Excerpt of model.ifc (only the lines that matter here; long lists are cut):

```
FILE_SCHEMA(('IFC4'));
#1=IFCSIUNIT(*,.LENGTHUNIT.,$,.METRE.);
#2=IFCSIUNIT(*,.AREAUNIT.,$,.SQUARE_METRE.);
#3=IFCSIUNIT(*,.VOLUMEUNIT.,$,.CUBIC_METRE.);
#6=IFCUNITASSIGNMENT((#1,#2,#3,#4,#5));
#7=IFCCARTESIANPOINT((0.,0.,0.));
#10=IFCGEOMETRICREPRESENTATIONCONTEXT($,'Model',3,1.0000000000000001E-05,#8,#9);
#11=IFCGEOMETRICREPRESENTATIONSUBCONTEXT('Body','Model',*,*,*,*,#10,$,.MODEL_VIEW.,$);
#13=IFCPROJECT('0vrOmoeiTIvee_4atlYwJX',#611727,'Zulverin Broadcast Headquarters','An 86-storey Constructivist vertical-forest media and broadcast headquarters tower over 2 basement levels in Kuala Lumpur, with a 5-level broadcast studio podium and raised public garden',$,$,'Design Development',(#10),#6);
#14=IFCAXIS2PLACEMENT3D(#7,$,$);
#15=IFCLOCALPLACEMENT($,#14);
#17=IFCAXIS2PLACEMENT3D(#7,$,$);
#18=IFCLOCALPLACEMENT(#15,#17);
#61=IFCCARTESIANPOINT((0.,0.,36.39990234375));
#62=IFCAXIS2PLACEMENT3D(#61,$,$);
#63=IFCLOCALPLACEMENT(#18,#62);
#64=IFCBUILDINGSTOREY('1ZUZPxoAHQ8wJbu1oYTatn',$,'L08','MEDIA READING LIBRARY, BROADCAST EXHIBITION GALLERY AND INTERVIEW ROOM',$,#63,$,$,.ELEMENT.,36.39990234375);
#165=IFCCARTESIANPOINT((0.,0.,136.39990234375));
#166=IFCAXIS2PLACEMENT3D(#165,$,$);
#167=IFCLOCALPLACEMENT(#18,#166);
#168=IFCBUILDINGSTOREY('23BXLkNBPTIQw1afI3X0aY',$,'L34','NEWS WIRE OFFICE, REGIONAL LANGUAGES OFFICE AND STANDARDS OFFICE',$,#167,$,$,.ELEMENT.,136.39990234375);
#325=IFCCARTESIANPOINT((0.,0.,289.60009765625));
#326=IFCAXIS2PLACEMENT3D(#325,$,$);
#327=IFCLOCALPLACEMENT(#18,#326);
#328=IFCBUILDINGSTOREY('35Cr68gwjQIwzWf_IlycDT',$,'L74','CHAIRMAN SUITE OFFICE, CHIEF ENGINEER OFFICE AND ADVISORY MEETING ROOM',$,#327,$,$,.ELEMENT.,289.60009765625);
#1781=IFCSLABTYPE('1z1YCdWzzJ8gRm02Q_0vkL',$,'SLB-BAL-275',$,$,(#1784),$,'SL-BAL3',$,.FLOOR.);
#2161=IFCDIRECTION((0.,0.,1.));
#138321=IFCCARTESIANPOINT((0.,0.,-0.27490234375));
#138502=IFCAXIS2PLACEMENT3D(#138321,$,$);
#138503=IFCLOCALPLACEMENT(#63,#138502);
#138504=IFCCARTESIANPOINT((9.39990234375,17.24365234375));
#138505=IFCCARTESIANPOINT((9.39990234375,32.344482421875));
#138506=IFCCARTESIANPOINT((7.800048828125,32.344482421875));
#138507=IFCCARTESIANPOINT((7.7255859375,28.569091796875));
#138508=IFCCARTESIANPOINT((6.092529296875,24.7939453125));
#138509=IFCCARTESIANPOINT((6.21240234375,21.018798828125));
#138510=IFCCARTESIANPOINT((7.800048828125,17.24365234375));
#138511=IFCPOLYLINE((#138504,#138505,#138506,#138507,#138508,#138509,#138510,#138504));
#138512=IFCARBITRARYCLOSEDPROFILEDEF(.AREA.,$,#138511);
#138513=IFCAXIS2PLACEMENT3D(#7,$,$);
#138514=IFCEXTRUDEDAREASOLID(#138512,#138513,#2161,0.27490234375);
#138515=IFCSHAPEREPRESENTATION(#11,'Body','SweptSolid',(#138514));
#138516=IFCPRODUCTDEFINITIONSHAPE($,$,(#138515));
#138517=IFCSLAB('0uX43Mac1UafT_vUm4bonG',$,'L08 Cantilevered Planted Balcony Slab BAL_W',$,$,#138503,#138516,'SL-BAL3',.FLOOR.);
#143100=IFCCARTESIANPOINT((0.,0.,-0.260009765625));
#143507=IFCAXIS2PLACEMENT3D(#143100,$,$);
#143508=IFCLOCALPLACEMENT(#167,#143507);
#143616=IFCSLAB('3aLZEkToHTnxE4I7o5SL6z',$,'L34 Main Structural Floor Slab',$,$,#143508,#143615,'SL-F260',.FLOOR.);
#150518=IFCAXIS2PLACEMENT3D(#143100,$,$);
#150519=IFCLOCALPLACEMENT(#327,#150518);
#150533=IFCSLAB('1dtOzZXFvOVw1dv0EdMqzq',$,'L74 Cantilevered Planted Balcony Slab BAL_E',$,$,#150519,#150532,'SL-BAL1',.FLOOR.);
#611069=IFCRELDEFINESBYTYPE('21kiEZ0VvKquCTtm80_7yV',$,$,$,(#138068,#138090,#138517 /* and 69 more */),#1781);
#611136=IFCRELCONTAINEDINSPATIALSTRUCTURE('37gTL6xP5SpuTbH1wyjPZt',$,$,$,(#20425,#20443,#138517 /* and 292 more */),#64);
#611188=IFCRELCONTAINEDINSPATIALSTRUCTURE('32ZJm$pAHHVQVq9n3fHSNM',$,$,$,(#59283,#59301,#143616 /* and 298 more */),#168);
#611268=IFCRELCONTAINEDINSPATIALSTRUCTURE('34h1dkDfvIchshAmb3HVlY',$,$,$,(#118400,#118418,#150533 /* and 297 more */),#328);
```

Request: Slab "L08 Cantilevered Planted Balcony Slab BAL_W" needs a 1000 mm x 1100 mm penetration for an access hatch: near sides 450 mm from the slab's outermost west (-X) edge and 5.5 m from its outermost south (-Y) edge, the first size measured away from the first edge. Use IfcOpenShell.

```python
import numpy as np
import ifcopenshell
import ifcopenshell.api.feature
import ifcopenshell.api.geometry
import ifcopenshell.api.root
import ifcopenshell.geom
import ifcopenshell.util.placement
import ifcopenshell.util.representation
import ifcopenshell.util.shape
import ifcopenshell.util.unit

model = ifcopenshell.open("model.ifc")
unit_scale = ifcopenshell.util.unit.calculate_unit_scale(model)
settings = ifcopenshell.geom.settings()


def volume(element):
    """Net volume in cubic metres, openings subtracted."""
    shape = ifcopenshell.geom.create_shape(settings, element)
    return ifcopenshell.util.shape.get_volume(shape.geometry)


slab = model.by_guid("0uX43Mac1UafT_vUm4bonG")
before = volume(slab)

# Extent in the slab's own axes, in metres. The edges named are its -X and -Y sides.
slab_shape = ifcopenshell.geom.create_shape(settings, slab)
vertices = ifcopenshell.util.shape.get_vertices(slab_shape.geometry)
x_min, y_min, bottom = vertices.min(axis=0)
top = vertices[:, 2].max()

opening = ifcopenshell.api.root.create_entity(model, ifc_class="IfcOpeningElement", name="Access hatch opening", predefined_type="OPENING")
context = ifcopenshell.util.representation.get_context(model, "Model", "Body", "MODEL_VIEW")
width, depth = 1, 1.1
outline = [(0.0, 0.0), (width, 0.0), (width, depth), (0.0, depth), (0.0, 0.0)]
# Overshoot both faces by 50 mm so the cut is clean.
shape = ifcopenshell.api.geometry.add_slab_representation(
    model, context=context, depth=top - bottom + 0.1, polyline=outline
)
ifcopenshell.api.geometry.assign_representation(model, product=opening, representation=shape)

matrix = ifcopenshell.util.placement.get_local_placement(slab.ObjectPlacement)
matrix[:, 3] = matrix @ np.append(np.array([x_min + 0.45, y_min + 5.5, bottom - 0.05]) / unit_scale, 1.0)
ifcopenshell.api.geometry.edit_object_placement(model, product=opening, matrix=matrix, is_si=False)
ifcopenshell.api.feature.add_feature(model, feature=opening, element=slab)

after = volume(slab)

print(f"slab volume {before:.3f} -> {after:.3f} m3")

model.write("model_edited.ifc")
```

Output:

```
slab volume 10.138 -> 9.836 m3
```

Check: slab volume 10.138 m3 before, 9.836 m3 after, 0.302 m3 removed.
